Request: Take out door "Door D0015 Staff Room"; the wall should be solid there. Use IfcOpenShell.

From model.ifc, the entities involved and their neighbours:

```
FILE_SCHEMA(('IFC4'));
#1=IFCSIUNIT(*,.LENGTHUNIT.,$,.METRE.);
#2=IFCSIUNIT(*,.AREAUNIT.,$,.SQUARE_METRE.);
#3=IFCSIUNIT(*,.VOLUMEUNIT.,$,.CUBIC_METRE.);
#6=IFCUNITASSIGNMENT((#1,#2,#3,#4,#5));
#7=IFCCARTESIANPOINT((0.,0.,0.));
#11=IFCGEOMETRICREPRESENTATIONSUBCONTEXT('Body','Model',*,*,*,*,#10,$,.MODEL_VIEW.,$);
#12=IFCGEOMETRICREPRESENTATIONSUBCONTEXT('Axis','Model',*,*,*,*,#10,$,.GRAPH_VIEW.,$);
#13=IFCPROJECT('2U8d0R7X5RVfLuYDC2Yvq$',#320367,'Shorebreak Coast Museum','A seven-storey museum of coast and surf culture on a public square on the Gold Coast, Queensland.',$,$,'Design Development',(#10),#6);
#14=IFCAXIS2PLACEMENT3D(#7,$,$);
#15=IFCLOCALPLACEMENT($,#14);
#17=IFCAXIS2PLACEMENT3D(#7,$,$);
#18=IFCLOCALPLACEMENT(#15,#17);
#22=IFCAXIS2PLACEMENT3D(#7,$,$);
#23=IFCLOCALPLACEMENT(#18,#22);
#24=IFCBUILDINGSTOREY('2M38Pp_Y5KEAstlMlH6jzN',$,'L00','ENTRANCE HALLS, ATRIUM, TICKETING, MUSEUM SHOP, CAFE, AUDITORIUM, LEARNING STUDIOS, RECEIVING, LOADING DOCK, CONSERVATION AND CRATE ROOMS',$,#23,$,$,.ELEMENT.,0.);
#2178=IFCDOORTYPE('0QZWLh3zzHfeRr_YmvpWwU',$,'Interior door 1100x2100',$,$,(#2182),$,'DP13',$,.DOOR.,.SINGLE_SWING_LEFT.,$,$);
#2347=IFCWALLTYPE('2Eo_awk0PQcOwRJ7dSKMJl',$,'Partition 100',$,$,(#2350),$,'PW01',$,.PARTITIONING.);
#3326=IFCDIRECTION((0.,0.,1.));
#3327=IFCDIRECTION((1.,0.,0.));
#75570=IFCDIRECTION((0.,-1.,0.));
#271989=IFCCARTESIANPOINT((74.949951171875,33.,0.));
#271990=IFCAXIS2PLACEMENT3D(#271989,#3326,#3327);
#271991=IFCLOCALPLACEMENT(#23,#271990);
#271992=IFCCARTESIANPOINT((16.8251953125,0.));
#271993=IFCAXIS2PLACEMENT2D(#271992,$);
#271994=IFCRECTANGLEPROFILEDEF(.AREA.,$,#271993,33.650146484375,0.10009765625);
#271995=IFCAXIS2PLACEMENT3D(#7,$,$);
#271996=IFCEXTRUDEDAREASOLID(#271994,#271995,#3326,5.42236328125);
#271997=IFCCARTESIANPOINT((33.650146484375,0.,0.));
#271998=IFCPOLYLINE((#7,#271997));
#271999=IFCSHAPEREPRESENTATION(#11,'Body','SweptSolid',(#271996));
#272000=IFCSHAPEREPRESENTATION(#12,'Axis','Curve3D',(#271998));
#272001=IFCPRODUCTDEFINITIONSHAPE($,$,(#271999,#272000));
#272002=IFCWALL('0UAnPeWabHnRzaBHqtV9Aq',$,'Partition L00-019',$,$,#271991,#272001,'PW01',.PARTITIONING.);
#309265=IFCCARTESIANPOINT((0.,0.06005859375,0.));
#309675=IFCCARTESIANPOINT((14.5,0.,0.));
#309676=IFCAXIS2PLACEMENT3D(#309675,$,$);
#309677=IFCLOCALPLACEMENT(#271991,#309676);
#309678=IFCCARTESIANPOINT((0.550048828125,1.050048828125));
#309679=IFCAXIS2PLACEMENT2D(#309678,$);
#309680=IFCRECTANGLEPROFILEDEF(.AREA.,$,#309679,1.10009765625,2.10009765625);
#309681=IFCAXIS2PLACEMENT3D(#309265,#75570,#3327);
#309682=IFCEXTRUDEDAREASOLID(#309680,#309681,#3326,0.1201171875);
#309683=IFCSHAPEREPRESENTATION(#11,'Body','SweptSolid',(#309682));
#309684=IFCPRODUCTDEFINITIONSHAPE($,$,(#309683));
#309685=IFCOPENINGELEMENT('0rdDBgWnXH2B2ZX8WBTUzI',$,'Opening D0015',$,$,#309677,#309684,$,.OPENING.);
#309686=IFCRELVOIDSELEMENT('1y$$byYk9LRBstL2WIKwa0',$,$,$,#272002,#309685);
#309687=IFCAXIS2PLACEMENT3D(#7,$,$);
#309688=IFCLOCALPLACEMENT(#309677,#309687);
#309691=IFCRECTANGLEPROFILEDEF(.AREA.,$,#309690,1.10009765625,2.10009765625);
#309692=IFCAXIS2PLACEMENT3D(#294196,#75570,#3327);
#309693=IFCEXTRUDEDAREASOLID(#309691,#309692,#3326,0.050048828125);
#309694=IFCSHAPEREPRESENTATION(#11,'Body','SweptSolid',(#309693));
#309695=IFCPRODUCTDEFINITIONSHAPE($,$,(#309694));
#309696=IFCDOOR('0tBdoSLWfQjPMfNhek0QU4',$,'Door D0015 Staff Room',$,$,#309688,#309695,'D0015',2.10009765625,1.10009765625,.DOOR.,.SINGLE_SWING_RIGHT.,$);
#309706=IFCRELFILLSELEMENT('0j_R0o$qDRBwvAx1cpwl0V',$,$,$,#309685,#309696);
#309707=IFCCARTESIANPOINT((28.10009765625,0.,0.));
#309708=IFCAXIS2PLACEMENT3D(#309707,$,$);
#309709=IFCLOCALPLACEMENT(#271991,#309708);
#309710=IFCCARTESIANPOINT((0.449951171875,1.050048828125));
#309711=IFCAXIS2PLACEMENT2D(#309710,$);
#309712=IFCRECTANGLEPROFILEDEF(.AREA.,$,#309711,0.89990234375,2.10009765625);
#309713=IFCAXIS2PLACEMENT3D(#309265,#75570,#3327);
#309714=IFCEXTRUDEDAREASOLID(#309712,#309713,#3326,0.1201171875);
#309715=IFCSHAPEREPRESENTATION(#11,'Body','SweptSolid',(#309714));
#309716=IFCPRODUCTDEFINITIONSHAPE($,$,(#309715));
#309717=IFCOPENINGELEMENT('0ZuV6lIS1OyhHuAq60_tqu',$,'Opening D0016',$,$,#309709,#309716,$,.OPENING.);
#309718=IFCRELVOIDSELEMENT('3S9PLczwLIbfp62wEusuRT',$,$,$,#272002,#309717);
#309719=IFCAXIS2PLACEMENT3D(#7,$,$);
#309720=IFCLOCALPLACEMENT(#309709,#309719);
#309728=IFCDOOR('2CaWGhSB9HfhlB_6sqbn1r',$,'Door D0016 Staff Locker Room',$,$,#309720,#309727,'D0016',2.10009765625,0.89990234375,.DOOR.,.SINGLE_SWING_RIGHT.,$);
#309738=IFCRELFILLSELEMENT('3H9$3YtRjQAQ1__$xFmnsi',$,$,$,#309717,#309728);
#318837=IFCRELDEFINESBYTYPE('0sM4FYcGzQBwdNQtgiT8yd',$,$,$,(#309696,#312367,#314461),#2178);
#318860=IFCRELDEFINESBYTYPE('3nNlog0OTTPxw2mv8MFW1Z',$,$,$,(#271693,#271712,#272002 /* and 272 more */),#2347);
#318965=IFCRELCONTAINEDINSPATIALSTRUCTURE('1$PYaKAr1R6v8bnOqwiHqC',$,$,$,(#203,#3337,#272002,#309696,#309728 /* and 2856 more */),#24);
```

```python
import ifcopenshell
import ifcopenshell.api.feature
import ifcopenshell.api.root
import ifcopenshell.geom
import ifcopenshell.util.shape

model = ifcopenshell.open("model.ifc")
settings = ifcopenshell.geom.settings()


def volume(element):
    """Net volume in cubic metres, openings subtracted."""
    shape = ifcopenshell.geom.create_shape(settings, element)
    return ifcopenshell.util.shape.get_volume(shape.geometry)


door = model.by_id(309696)
opening = door.FillsVoids[0].RelatingOpeningElement
wall = opening.VoidsElements[0].RelatingBuildingElement
before = volume(wall)

ifcopenshell.api.root.remove_product(model, product=door)
ifcopenshell.api.feature.remove_feature(model, feature=opening)

after = volume(wall)

print(f"wall volume {before:.3f} -> {after:.3f} m3")

model.write("model_v2.ifc")
```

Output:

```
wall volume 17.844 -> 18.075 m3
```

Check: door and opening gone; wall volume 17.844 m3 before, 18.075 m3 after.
